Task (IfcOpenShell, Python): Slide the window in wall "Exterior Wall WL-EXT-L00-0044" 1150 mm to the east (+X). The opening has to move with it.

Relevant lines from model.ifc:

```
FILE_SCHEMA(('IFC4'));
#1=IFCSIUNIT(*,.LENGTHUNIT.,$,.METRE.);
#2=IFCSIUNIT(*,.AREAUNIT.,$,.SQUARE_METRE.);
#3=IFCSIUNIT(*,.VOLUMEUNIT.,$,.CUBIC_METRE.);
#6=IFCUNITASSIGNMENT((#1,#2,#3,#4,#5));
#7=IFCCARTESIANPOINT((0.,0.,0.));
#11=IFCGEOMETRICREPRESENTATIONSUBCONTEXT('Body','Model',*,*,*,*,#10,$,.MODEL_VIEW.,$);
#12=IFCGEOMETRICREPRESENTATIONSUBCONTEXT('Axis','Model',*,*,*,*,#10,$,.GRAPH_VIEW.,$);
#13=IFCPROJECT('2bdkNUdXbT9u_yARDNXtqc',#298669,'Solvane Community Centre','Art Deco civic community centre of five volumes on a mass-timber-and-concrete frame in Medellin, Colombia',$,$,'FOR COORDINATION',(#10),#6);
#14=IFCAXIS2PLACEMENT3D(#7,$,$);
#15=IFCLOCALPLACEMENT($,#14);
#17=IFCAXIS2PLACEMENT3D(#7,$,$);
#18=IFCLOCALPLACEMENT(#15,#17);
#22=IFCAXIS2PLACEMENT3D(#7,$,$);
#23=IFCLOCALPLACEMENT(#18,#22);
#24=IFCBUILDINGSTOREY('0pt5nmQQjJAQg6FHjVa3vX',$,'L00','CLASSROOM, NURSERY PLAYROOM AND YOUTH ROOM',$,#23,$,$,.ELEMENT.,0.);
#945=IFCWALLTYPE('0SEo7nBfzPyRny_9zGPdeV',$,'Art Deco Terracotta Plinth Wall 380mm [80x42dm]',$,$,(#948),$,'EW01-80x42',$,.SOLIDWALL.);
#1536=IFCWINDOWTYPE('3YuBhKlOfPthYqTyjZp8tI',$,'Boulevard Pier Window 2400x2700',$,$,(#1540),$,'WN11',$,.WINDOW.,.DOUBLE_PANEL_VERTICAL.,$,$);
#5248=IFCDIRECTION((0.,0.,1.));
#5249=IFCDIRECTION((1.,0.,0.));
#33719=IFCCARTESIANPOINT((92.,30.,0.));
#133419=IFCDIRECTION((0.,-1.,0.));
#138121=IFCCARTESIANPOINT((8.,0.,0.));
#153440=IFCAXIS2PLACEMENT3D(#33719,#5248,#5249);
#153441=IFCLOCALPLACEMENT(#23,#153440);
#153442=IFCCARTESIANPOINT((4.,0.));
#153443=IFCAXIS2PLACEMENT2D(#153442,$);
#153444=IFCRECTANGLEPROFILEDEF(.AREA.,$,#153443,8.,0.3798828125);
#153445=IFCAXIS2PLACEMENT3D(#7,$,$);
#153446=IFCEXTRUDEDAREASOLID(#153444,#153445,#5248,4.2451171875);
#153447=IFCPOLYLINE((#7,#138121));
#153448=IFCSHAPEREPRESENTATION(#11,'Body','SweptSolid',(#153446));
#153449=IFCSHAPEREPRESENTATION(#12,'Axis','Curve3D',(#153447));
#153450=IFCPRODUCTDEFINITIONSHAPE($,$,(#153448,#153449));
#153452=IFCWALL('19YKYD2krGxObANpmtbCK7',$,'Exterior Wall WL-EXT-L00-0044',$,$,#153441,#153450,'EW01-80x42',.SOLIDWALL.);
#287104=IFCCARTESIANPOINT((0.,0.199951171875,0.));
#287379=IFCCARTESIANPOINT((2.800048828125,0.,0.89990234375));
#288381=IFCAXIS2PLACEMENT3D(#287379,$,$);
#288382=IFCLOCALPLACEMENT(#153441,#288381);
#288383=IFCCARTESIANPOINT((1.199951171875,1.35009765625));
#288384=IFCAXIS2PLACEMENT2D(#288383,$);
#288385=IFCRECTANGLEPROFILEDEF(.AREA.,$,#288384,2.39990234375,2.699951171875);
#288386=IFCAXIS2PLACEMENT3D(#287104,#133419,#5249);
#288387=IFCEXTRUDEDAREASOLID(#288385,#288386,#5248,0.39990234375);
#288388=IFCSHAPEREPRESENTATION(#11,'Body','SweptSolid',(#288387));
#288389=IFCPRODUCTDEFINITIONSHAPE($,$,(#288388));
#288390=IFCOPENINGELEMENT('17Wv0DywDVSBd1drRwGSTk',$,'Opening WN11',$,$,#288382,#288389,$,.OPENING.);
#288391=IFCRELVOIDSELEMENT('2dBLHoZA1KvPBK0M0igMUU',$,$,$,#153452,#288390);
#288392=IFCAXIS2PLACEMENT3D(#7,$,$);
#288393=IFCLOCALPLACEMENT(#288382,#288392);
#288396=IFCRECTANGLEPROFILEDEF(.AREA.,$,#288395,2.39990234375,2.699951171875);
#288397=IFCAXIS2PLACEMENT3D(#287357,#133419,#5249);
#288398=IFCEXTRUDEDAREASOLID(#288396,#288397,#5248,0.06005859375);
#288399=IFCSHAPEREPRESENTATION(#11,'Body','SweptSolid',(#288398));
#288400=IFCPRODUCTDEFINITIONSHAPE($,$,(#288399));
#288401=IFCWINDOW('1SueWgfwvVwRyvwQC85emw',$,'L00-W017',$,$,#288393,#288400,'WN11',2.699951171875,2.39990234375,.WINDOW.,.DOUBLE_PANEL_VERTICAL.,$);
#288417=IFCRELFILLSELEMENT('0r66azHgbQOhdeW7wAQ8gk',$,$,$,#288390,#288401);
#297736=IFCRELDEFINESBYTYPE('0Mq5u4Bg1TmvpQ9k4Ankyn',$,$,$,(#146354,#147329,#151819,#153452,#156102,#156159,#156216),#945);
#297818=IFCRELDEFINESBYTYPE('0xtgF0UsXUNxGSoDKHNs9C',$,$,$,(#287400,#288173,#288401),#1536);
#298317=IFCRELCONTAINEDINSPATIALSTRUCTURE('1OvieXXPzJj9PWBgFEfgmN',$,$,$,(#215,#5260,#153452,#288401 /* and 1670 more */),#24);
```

```python
import ifcopenshell
import ifcopenshell.api.geometry
import ifcopenshell.util.placement
import ifcopenshell.util.unit

model = ifcopenshell.open("model.ifc")
unit_scale = ifcopenshell.util.unit.calculate_unit_scale(model)

window = model.by_id(288401)
opening = window.FillsVoids[0].RelatingOpeningElement
wall = opening.VoidsElements[0].RelatingBuildingElement

wall_matrix = ifcopenshell.util.placement.get_local_placement(wall.ObjectPlacement)
shift = wall_matrix[:3, 0] * 1.15 / unit_scale
before = ifcopenshell.util.placement.get_local_placement(window.ObjectPlacement)[:3, 3].copy()

# The window is placed relative to its opening, so it follows when the opening moves.
matrix = ifcopenshell.util.placement.get_local_placement(opening.ObjectPlacement)
matrix[:3, 3] += shift
ifcopenshell.api.geometry.edit_object_placement(
    model, product=opening, matrix=matrix, is_si=False, should_transform_children=True
)

after = ifcopenshell.util.placement.get_local_placement(window.ObjectPlacement)[:3, 3]
print("window moved by", (after - before).round(3) + 0.0)

model.write("model_edited.ifc")
```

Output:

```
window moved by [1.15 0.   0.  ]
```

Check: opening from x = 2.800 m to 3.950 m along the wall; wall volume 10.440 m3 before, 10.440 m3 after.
